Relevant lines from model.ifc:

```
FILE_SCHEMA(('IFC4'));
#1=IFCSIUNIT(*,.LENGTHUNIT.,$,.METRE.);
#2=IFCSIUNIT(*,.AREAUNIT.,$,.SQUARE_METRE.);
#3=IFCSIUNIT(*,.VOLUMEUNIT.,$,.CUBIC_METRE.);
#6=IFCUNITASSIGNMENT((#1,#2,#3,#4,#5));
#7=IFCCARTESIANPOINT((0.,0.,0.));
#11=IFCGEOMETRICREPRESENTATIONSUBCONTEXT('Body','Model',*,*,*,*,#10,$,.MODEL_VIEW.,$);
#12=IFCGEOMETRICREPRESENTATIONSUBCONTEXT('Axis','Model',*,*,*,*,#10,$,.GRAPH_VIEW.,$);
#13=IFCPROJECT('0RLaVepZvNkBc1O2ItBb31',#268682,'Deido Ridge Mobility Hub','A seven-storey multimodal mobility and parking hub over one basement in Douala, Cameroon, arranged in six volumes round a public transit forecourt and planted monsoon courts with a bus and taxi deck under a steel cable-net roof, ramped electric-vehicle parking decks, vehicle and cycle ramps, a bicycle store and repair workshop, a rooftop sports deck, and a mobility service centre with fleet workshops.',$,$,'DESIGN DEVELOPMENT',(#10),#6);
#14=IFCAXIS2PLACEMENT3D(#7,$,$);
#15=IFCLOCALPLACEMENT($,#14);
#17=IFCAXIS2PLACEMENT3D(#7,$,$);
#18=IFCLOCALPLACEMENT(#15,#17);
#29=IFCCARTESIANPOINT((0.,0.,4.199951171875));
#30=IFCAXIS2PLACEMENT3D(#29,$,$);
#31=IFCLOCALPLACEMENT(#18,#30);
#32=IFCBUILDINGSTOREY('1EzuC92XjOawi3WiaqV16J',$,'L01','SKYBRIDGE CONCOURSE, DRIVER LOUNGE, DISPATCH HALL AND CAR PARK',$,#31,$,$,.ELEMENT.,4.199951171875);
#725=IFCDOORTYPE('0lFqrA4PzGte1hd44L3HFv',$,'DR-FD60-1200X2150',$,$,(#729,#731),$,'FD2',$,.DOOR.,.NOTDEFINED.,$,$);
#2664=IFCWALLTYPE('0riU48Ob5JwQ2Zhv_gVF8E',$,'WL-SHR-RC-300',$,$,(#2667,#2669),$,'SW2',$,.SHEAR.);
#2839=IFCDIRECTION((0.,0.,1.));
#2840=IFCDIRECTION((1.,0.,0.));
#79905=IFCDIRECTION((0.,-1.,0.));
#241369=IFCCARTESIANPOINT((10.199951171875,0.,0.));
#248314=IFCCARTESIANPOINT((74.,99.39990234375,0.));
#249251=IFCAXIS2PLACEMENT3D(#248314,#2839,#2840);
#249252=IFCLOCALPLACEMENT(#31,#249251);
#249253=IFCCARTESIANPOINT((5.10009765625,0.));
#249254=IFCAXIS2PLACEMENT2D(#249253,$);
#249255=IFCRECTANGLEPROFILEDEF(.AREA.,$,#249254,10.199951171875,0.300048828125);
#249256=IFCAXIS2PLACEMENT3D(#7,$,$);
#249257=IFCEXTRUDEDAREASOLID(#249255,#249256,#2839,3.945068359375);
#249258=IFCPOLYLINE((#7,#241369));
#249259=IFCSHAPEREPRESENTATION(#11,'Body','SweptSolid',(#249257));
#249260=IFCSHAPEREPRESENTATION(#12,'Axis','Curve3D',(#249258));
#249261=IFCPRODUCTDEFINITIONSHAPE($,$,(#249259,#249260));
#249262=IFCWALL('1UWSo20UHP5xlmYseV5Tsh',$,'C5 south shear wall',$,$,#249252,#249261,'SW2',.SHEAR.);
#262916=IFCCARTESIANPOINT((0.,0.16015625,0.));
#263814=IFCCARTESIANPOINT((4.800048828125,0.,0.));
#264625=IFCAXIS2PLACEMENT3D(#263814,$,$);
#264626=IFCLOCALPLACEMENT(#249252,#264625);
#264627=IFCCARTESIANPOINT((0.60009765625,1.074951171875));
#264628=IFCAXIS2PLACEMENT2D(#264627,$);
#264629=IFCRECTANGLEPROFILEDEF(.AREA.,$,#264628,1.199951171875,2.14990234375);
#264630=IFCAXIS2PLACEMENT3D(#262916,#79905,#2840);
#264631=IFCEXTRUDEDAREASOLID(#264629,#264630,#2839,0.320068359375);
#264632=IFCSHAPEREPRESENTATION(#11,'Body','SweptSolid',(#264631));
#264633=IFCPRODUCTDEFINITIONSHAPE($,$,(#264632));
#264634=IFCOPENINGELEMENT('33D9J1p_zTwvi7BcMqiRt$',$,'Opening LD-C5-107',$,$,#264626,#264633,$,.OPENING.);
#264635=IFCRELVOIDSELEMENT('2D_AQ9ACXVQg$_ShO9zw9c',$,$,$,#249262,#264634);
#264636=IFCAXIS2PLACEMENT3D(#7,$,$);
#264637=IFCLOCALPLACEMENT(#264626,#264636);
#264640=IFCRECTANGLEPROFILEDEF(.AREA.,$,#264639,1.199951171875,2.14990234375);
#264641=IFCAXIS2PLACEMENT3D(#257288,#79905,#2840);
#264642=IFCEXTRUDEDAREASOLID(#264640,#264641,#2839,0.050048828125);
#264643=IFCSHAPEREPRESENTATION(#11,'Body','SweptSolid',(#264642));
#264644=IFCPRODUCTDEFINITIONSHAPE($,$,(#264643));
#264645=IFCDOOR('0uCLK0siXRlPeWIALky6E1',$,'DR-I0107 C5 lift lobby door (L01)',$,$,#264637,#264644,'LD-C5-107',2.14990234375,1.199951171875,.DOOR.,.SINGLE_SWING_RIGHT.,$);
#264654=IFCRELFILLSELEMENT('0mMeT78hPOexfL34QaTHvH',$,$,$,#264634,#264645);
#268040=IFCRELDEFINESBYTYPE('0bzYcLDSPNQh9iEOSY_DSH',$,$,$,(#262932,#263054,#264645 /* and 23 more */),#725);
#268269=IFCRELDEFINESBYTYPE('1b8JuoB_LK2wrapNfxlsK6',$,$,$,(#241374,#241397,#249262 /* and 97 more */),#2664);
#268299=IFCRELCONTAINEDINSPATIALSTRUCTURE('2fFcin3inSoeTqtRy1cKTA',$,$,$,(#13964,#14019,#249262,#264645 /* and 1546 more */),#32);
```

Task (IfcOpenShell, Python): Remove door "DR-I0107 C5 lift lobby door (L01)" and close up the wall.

```python
import ifcopenshell
import ifcopenshell.api.feature
import ifcopenshell.api.root
import ifcopenshell.geom
import ifcopenshell.util.shape

model = ifcopenshell.open("model.ifc")
settings = ifcopenshell.geom.settings()


def volume(element):
    """Net volume in cubic metres, openings subtracted."""
    shape = ifcopenshell.geom.create_shape(settings, element)
    return ifcopenshell.util.shape.get_volume(shape.geometry)


door = model.by_guid("0uCLK0siXRlPeWIALky6E1")
opening = door.FillsVoids[0].RelatingOpeningElement
wall = opening.VoidsElements[0].RelatingBuildingElement
before = volume(wall)

ifcopenshell.api.root.remove_product(model, product=door)
ifcopenshell.api.feature.remove_feature(model, feature=opening)

after = volume(wall)

print(f"wall volume {before:.3f} -> {after:.3f} m3")

model.write("model_v2.ifc")
```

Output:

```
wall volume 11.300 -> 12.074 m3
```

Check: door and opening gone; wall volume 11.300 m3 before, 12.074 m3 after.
